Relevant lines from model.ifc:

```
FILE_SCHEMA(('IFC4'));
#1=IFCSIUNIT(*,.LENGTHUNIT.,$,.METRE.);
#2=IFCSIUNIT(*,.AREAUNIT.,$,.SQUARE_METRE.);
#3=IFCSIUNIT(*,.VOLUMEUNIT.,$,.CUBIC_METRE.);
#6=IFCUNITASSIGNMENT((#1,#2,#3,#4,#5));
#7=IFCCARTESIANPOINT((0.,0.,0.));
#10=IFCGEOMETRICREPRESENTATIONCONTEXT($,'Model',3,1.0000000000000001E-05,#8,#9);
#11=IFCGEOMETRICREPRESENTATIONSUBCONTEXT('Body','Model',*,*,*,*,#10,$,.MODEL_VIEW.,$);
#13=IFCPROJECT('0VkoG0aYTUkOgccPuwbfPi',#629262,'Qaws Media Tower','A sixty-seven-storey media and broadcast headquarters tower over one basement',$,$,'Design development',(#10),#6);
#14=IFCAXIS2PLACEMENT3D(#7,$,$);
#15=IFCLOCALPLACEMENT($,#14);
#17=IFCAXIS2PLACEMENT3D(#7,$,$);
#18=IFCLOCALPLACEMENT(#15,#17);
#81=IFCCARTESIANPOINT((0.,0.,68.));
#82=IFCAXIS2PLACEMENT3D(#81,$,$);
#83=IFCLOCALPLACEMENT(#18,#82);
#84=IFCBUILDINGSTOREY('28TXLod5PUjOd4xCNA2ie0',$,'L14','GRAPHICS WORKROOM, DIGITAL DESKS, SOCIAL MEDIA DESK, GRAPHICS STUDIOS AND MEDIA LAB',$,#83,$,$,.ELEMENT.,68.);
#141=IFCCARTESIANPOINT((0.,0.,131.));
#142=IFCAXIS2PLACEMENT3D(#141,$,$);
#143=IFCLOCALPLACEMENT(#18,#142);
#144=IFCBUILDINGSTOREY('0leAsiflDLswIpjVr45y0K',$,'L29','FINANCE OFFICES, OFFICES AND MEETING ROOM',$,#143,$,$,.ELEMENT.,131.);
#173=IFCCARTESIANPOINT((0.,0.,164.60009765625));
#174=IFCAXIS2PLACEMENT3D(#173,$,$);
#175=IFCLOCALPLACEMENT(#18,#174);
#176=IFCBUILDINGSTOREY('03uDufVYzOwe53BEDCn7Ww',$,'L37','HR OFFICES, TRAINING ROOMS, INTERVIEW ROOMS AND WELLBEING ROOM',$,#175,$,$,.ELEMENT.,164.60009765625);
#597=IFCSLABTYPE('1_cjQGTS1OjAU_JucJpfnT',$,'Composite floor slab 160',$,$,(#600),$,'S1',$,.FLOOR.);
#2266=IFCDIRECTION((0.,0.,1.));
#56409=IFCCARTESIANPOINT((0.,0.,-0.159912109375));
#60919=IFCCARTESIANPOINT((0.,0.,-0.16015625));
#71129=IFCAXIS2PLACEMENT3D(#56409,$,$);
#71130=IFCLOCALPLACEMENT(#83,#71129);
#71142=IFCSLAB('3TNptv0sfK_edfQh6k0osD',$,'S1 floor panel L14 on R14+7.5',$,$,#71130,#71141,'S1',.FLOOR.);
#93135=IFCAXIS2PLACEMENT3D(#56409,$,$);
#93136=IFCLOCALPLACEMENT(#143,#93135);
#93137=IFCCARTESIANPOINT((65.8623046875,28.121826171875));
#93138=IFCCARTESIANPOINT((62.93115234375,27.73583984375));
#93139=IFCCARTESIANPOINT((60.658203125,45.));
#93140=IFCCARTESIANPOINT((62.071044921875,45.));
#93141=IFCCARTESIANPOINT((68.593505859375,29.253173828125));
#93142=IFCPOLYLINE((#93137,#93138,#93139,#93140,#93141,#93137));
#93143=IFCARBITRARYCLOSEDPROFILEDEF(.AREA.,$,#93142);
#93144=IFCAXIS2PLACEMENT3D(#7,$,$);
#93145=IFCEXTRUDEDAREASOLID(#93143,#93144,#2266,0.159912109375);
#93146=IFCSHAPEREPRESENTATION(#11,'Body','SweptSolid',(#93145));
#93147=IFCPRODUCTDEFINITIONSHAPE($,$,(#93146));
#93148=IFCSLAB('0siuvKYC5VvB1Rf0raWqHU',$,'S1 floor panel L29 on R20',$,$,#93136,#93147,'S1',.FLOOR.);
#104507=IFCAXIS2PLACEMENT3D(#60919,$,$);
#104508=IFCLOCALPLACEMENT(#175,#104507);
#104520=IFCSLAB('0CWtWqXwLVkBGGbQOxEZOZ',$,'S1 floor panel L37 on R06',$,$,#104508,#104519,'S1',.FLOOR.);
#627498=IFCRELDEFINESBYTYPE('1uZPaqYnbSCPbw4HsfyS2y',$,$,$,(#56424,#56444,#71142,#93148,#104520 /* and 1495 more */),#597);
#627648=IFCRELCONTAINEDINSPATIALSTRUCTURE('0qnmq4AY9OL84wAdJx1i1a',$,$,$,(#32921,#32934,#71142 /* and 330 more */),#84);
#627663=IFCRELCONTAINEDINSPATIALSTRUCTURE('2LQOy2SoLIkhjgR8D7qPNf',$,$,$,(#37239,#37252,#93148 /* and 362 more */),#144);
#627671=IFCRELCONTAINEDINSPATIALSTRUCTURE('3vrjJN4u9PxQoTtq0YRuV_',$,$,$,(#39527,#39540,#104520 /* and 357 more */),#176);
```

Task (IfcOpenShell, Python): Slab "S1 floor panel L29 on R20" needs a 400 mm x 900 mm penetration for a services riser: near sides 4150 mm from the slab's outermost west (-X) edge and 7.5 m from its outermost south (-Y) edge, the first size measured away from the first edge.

```python
import numpy as np
import ifcopenshell
import ifcopenshell.api.feature
import ifcopenshell.api.geometry
import ifcopenshell.api.root
import ifcopenshell.geom
import ifcopenshell.util.placement
import ifcopenshell.util.representation
import ifcopenshell.util.shape
import ifcopenshell.util.unit

model = ifcopenshell.open("model.ifc")
unit_scale = ifcopenshell.util.unit.calculate_unit_scale(model)
settings = ifcopenshell.geom.settings()


def volume(element):
    """Net volume in cubic metres, openings subtracted."""
    shape = ifcopenshell.geom.create_shape(settings, element)
    return ifcopenshell.util.shape.get_volume(shape.geometry)


slab = model.by_guid("0siuvKYC5VvB1Rf0raWqHU")
before = volume(slab)

# Extent in the slab's own axes, in metres. The edges named are its -X and -Y sides.
slab_shape = ifcopenshell.geom.create_shape(settings, slab)
vertices = ifcopenshell.util.shape.get_vertices(slab_shape.geometry)
x_min, y_min, bottom = vertices.min(axis=0)
top = vertices[:, 2].max()

opening = ifcopenshell.api.root.create_entity(model, ifc_class="IfcOpeningElement", name="Services riser opening", predefined_type="OPENING")
context = ifcopenshell.util.representation.get_context(model, "Model", "Body", "MODEL_VIEW")
width, depth = 0.4, 0.9
outline = [(0.0, 0.0), (width, 0.0), (width, depth), (0.0, depth), (0.0, 0.0)]
# Overshoot both faces by 50 mm so the cut is clean.
shape = ifcopenshell.api.geometry.add_slab_representation(
    model, context=context, depth=top - bottom + 0.1, polyline=outline
)
ifcopenshell.api.geometry.assign_representation(model, product=opening, representation=shape)

matrix = ifcopenshell.util.placement.get_local_placement(slab.ObjectPlacement)
matrix[:, 3] = matrix @ np.append(np.array([x_min + 4.15, y_min + 7.5, bottom - 0.05]) / unit_scale, 1.0)
ifcopenshell.api.geometry.edit_object_placement(model, product=opening, matrix=matrix, is_si=False)
ifcopenshell.api.feature.add_feature(model, feature=opening, element=slab)

after = volume(slab)

print(f"slab volume {before:.3f} -> {after:.3f} m3")

model.write("model_rev.ifc")
```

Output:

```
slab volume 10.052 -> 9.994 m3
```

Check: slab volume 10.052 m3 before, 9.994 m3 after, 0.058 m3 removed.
